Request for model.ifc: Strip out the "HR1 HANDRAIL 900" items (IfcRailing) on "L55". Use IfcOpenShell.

First a look at what the model holds.

```python
import ifcopenshell
import ifcopenshell.util.element

model = ifcopenshell.open("model.ifc")
print(model.schema)
storey = next(s for s in model.by_type("IfcBuildingStorey") if s.Name == "L55")
railings = [e for e in ifcopenshell.util.element.get_decomposition(storey) if e.is_a("IfcRailing")]
seen = {}
for e in railings:
    element_type = ifcopenshell.util.element.get_type(e)
    name = element_type.Name if element_type not in (None, e) else None
    seen[name] = seen.get(name, 0) + 1
for name, count in sorted(seen.items(), key=str):
    print(count, "x", name)
```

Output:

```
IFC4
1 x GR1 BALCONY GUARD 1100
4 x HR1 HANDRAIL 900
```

```python
import ifcopenshell
import ifcopenshell.api.root
import ifcopenshell.util.element

model = ifcopenshell.open("model.ifc")

storey = next(s for s in model.by_type("IfcBuildingStorey") if s.Name == "L55")
railings = [e for e in ifcopenshell.util.element.get_decomposition(storey) if e.is_a("IfcRailing")]
targets = [e for e in railings if (t := ifcopenshell.util.element.get_type(e)) not in (None, e) and t.Name == "HR1 HANDRAIL 900"]

for e in targets:
    ifcopenshell.api.root.remove_product(model, product=e)
print(len(targets), "removed")

model.write("model_updated.ifc")
```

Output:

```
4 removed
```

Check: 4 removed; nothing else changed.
